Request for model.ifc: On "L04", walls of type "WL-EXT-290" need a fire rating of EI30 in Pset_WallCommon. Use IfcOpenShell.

First a look at what the model holds.

```python
import ifcopenshell
import ifcopenshell.util.element

model = ifcopenshell.open("model.ifc")
print(model.schema)
storey = next(s for s in model.by_type("IfcBuildingStorey") if s.Name == "L04")
walls = [e for e in ifcopenshell.util.element.get_decomposition(storey) if e.is_a("IfcWall")]
seen = {}
for e in walls:
    element_type = ifcopenshell.util.element.get_type(e)
    key = (element_type.Name if element_type != e and element_type else None, ifcopenshell.util.element.get_pset(e, "Pset_WallCommon", "FireRating"))
    seen[key] = seen.get(key, 0) + 1
for (name, value), count in sorted(seen.items(), key=str):
    print(count, "x", name, "|", value)
```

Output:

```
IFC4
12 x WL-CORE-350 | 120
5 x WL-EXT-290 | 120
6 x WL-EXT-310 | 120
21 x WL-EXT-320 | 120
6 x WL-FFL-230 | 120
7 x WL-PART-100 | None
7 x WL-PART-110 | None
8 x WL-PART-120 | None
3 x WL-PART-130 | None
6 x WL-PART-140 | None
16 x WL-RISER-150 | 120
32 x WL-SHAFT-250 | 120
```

```python
import ifcopenshell
import ifcopenshell.api.pset
import ifcopenshell.util.element

model = ifcopenshell.open("model.ifc")

storey = next(s for s in model.by_type("IfcBuildingStorey") if s.Name == "L04")
walls = [e for e in ifcopenshell.util.element.get_decomposition(storey) if e.is_a("IfcWall")]

count = 0
for e in walls:
    element_type = ifcopenshell.util.element.get_type(e)
    if element_type in (None, e) or element_type.Name != "WL-EXT-290":
        continue
    # add_pset returns the element's existing set when there is one.
    pset = ifcopenshell.api.pset.add_pset(model, product=e, name="Pset_WallCommon")
    ifcopenshell.api.pset.edit_pset(model, pset=pset, properties={"FireRating": "EI30"})
    count += 1

print(count, "walls updated")

model.write("model-out.ifc")
```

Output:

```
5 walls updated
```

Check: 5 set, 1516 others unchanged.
